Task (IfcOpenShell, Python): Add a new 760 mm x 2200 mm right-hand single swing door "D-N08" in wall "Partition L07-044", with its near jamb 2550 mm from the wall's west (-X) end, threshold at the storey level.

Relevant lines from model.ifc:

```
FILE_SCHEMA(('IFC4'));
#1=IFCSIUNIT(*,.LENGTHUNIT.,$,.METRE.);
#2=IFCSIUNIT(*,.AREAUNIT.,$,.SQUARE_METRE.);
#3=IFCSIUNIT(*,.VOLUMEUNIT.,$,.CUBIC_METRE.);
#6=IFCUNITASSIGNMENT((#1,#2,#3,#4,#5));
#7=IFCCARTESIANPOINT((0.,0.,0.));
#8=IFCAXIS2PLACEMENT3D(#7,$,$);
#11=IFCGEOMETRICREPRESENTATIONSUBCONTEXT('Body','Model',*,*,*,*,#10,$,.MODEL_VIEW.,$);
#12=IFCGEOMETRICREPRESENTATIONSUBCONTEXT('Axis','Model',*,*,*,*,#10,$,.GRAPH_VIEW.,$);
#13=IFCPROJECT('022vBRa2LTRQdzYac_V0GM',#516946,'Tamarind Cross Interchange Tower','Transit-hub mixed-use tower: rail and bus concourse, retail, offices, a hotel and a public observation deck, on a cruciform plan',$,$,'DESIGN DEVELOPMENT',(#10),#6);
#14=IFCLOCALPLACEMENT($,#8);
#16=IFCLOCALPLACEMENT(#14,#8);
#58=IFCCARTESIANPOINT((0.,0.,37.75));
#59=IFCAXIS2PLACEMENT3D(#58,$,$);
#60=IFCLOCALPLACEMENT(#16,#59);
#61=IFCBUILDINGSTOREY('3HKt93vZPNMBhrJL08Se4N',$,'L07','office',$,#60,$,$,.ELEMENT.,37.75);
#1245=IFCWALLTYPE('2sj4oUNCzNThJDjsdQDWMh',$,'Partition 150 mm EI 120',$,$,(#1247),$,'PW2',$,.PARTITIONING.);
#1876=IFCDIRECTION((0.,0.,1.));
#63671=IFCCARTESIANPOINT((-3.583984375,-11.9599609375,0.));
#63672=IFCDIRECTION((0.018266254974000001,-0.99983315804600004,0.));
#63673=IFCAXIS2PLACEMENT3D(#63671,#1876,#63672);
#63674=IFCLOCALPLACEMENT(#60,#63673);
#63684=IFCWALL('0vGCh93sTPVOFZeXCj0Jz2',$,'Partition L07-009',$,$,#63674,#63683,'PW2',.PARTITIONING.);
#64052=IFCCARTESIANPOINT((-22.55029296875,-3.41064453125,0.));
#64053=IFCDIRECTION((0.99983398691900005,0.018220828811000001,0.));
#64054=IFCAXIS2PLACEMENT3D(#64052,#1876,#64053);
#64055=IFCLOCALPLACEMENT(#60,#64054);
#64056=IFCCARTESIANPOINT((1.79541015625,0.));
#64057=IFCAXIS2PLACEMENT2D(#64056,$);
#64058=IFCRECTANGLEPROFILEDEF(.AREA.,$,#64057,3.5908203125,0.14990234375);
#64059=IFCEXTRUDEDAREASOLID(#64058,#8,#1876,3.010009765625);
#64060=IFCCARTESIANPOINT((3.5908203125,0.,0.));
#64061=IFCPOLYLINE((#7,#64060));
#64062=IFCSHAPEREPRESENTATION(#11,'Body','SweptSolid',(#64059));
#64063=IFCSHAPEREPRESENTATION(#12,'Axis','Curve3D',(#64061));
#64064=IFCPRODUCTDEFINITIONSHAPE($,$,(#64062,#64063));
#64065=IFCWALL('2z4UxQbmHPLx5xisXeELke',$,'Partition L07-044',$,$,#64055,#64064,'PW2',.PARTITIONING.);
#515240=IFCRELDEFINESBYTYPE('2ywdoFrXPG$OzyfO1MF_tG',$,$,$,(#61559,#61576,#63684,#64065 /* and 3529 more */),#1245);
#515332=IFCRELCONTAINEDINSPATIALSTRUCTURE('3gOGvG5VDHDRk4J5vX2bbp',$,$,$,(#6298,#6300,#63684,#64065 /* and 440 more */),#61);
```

```python
import numpy as np
import ifcopenshell
import ifcopenshell.api.feature
import ifcopenshell.api.geometry
import ifcopenshell.api.root
import ifcopenshell.api.spatial
import ifcopenshell.geom
import ifcopenshell.util.element
import ifcopenshell.util.placement
import ifcopenshell.util.representation
import ifcopenshell.util.shape
import ifcopenshell.util.unit

model = ifcopenshell.open("model.ifc")
unit_scale = ifcopenshell.util.unit.calculate_unit_scale(model)
settings = ifcopenshell.geom.settings()


def volume(element):
    """Net volume in cubic metres, openings subtracted."""
    shape = ifcopenshell.geom.create_shape(settings, element)
    return ifcopenshell.util.shape.get_volume(shape.geometry)


wall = model.by_guid("2z4UxQbmHPLx5xisXeELke")
storey = ifcopenshell.util.element.get_container(wall, ifc_class="IfcBuildingStorey")
context = ifcopenshell.util.representation.get_context(model, "Model", "Body", "MODEL_VIEW")
before = volume(wall)

width, height, from_end, sill = 0.76, 2.2, 2.55, 0.0  # metres

# The wall runs along its own X axis, and the end named is its -X end.
wall_shape = ifcopenshell.geom.create_shape(settings, wall)
x, y, z = ifcopenshell.util.shape.get_vertices(wall_shape.geometry).T
start = x.min() + from_end
face, thickness = float(y.min()), float(y.max() - y.min())
wall_matrix = ifcopenshell.util.placement.get_local_placement(wall.ObjectPlacement)
level = ifcopenshell.util.placement.get_local_placement(storey.ObjectPlacement)[2, 3]


def in_wall(x, y):
    """Placement at x, y metres in the wall's axes, at sill height."""
    matrix = wall_matrix.copy()
    matrix[:, 3] = wall_matrix @ np.array([x / unit_scale, y / unit_scale, 0.0, 1.0])
    matrix[2, 3] = level + sill / unit_scale
    return matrix


# Opening: a box that overshoots both wall faces by 50 mm.
opening = ifcopenshell.api.root.create_entity(model, ifc_class="IfcOpeningElement", predefined_type="OPENING")
box = ifcopenshell.api.geometry.add_wall_representation(
    model, context=context, length=width, height=height, thickness=thickness + 0.1
)
ifcopenshell.api.geometry.assign_representation(model, product=opening, representation=box)
ifcopenshell.api.geometry.edit_object_placement(model, product=opening, matrix=in_wall(start, face - 0.05), is_si=False)
ifcopenshell.api.feature.add_feature(model, feature=opening, element=wall)

door = ifcopenshell.api.root.create_entity(model, ifc_class="IfcDoor", name="D-N08", predefined_type="DOOR")
door.OverallWidth, door.OverallHeight = width / unit_scale, height / unit_scale
door.OperationType = "SINGLE_SWING_RIGHT"
body = ifcopenshell.api.geometry.add_door_representation(
    model,
    context=context,
    overall_width=door.OverallWidth,
    overall_height=door.OverallHeight,
    operation_type="SINGLE_SWING_RIGHT",
    lining_properties={"LiningDepth": thickness / unit_scale, "ThresholdDepth": thickness / unit_scale},
)
ifcopenshell.api.geometry.assign_representation(model, product=door, representation=body)
ifcopenshell.api.spatial.assign_container(model, products=[door], relating_structure=storey)
ifcopenshell.api.feature.add_filling(model, opening=opening, element=door)

# The lining spans the wall, so the door starts at the wall face.
ifcopenshell.api.geometry.edit_object_placement(model, product=door, matrix=in_wall(start, face), is_si=False)

after = volume(wall)

print(f"wall volume {before:.3f} -> {after:.3f} m3")

model.write("model_v2.ifc")
```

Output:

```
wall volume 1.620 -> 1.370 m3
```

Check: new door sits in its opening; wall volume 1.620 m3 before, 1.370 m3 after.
